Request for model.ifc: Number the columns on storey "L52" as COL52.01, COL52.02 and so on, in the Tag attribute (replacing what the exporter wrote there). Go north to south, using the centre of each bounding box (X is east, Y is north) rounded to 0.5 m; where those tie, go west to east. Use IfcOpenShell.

First a look at what the model holds.

```python
import ifcopenshell
import ifcopenshell.util.element
import ifcopenshell.util.placement

model = ifcopenshell.open("model.ifc")
print(model.schema)
storey = next(s for s in model.by_type("IfcBuildingStorey") if s.Name == "L52")
columns = [e for e in ifcopenshell.util.element.get_decomposition(storey) if e.is_a("IfcColumn")]
for e in sorted(columns, key=lambda e: e.id()):
    origin = ifcopenshell.util.placement.get_local_placement(e.ObjectPlacement)[:3, 3]
    print(e.id(), e.Tag, e.Name, origin.round(2) + 0.0, sep=" | ")
```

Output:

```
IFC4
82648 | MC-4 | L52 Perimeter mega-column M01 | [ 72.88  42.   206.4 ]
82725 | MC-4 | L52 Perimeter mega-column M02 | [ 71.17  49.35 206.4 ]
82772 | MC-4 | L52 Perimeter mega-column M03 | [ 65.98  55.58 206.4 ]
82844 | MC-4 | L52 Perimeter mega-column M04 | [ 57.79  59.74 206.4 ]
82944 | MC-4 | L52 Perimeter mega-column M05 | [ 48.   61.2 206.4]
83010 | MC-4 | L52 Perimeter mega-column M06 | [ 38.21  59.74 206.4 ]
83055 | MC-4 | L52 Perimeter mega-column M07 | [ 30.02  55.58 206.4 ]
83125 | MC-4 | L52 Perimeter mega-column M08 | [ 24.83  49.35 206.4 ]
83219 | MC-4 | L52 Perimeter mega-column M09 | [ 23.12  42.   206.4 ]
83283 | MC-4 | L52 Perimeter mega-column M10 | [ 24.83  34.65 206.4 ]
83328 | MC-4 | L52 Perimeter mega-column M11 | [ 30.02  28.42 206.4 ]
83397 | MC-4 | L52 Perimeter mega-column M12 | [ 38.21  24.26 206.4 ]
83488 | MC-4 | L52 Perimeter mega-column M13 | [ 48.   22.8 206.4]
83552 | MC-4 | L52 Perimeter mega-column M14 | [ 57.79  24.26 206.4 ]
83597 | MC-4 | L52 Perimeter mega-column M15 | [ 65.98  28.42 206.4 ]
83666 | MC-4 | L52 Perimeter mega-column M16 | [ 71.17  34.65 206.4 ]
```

```python
import ifcopenshell
import ifcopenshell.geom
import ifcopenshell.util.element
import ifcopenshell.util.shape

model = ifcopenshell.open("model.ifc")
settings = ifcopenshell.geom.settings()
settings.set("use-world-coords", True)


def centre(element):
    shape = ifcopenshell.geom.create_shape(settings, element)
    return ifcopenshell.util.shape.get_bbox_centroid(shape.geometry)


storey = next(s for s in model.by_type("IfcBuildingStorey") if s.Name == "L52")
columns = [e for e in ifcopenshell.util.element.get_decomposition(storey) if e.is_a("IfcColumn")]

# Insertion points can sit at a corner or the storey origin, so sort by the geometry (in metres).
centres = {e: centre(e) for e in columns}
columns.sort(key=lambda e: (-round(centres[e][1] / 0.5), centres[e][0]))

for i, e in enumerate(columns, start=1):
    number = f"COL52.{i:02d}"
    e.Tag = number
    print(e.id(), number)

model.write("model_edited.ifc")
```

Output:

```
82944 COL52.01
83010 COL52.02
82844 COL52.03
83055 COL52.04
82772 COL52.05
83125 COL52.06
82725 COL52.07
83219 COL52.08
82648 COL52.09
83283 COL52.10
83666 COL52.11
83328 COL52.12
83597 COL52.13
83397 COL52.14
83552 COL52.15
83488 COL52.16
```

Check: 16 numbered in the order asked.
